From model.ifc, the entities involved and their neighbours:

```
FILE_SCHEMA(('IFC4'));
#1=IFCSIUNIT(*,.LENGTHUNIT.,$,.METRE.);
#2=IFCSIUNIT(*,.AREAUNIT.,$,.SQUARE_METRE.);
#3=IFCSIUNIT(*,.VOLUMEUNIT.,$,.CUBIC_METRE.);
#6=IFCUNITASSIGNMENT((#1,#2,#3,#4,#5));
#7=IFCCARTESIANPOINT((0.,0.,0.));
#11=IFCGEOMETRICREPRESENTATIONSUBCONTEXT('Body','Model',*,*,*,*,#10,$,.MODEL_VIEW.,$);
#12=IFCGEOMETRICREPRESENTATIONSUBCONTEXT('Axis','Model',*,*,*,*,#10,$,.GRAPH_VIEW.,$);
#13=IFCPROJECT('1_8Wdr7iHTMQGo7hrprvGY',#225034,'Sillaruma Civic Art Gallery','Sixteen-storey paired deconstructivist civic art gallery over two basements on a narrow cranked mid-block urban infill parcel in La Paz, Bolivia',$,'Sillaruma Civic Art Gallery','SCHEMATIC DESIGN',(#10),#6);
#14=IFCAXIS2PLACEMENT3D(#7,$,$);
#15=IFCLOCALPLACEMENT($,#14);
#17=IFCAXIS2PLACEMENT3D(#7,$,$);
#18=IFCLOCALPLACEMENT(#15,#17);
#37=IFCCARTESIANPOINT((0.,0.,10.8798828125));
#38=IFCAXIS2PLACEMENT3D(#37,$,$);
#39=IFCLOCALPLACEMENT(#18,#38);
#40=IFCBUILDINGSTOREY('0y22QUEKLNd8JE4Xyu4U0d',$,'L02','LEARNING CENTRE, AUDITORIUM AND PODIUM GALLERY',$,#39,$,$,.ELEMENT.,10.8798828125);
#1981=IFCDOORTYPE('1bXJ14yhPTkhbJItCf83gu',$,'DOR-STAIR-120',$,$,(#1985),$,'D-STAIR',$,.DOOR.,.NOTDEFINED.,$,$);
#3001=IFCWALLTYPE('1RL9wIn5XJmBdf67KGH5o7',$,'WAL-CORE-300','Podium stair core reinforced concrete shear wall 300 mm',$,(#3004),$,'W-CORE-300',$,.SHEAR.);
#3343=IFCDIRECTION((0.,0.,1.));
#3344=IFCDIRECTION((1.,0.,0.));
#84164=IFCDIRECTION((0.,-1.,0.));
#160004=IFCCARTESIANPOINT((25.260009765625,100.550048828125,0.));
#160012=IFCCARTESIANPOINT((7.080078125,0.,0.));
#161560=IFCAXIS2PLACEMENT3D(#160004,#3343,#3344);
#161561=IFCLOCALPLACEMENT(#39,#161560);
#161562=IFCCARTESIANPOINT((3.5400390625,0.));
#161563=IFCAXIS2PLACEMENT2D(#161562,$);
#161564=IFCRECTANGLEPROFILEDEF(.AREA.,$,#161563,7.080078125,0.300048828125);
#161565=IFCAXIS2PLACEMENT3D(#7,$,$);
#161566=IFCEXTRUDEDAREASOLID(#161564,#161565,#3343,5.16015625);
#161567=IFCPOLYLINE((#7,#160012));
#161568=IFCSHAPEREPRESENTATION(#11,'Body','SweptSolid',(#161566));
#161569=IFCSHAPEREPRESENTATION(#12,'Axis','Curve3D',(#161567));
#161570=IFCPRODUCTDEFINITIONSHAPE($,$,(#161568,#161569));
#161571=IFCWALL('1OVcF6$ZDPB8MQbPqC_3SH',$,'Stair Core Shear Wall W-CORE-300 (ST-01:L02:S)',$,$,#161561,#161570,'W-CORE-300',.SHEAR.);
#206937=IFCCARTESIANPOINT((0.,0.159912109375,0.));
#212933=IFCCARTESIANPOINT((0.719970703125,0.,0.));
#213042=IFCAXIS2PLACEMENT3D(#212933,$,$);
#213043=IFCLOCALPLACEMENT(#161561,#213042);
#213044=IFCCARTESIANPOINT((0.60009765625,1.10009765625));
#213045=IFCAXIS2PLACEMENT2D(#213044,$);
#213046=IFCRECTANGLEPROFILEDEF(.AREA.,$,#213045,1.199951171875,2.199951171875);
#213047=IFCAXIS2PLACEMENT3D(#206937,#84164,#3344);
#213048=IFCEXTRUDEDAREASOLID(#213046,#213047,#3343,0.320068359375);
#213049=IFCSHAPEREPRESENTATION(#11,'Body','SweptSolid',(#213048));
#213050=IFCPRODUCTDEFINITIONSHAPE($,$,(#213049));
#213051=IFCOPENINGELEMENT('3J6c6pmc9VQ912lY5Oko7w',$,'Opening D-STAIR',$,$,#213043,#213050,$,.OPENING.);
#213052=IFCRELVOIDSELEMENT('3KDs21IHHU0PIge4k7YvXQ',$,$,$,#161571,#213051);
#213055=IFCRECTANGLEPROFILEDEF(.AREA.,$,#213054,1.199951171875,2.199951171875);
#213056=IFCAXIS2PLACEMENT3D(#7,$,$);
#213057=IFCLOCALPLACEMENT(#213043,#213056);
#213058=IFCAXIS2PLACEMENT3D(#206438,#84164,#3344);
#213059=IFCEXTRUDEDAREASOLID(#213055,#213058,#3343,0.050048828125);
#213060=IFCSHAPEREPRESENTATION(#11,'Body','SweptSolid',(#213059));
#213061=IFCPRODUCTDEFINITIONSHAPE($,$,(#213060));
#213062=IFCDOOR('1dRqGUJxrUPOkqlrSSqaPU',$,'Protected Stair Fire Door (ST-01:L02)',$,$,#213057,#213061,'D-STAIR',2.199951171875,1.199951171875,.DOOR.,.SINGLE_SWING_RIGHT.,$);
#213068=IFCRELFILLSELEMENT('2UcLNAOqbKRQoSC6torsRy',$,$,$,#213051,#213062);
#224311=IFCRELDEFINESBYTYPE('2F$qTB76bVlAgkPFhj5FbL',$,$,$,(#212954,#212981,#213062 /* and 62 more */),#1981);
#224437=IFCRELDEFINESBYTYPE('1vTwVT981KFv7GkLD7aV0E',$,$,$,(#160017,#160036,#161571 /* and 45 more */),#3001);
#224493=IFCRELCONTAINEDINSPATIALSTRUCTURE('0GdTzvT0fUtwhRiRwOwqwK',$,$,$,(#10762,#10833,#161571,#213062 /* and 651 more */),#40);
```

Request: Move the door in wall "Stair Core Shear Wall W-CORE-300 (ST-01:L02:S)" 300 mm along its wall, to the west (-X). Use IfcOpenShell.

```python
import ifcopenshell
import ifcopenshell.api.geometry
import ifcopenshell.util.placement

model = ifcopenshell.open("model.ifc")

door = model.by_id(213062)
opening = door.FillsVoids[0].RelatingOpeningElement
wall = opening.VoidsElements[0].RelatingBuildingElement

wall_matrix = ifcopenshell.util.placement.get_local_placement(wall.ObjectPlacement)
shift = wall_matrix[:3, 0] * -0.3
before = ifcopenshell.util.placement.get_local_placement(door.ObjectPlacement)[:3, 3].copy()

# The door is placed relative to its opening, so it follows when the opening moves.
matrix = ifcopenshell.util.placement.get_local_placement(opening.ObjectPlacement)
matrix[:3, 3] += shift
ifcopenshell.api.geometry.edit_object_placement(
    model, product=opening, matrix=matrix, is_si=False, should_transform_children=True
)

after = ifcopenshell.util.placement.get_local_placement(door.ObjectPlacement)[:3, 3]
print("door moved by", (after - before).round(3) + 0.0)

model.write("model_updated.ifc")
```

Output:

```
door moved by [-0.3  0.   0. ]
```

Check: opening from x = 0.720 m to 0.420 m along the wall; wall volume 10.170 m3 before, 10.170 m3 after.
